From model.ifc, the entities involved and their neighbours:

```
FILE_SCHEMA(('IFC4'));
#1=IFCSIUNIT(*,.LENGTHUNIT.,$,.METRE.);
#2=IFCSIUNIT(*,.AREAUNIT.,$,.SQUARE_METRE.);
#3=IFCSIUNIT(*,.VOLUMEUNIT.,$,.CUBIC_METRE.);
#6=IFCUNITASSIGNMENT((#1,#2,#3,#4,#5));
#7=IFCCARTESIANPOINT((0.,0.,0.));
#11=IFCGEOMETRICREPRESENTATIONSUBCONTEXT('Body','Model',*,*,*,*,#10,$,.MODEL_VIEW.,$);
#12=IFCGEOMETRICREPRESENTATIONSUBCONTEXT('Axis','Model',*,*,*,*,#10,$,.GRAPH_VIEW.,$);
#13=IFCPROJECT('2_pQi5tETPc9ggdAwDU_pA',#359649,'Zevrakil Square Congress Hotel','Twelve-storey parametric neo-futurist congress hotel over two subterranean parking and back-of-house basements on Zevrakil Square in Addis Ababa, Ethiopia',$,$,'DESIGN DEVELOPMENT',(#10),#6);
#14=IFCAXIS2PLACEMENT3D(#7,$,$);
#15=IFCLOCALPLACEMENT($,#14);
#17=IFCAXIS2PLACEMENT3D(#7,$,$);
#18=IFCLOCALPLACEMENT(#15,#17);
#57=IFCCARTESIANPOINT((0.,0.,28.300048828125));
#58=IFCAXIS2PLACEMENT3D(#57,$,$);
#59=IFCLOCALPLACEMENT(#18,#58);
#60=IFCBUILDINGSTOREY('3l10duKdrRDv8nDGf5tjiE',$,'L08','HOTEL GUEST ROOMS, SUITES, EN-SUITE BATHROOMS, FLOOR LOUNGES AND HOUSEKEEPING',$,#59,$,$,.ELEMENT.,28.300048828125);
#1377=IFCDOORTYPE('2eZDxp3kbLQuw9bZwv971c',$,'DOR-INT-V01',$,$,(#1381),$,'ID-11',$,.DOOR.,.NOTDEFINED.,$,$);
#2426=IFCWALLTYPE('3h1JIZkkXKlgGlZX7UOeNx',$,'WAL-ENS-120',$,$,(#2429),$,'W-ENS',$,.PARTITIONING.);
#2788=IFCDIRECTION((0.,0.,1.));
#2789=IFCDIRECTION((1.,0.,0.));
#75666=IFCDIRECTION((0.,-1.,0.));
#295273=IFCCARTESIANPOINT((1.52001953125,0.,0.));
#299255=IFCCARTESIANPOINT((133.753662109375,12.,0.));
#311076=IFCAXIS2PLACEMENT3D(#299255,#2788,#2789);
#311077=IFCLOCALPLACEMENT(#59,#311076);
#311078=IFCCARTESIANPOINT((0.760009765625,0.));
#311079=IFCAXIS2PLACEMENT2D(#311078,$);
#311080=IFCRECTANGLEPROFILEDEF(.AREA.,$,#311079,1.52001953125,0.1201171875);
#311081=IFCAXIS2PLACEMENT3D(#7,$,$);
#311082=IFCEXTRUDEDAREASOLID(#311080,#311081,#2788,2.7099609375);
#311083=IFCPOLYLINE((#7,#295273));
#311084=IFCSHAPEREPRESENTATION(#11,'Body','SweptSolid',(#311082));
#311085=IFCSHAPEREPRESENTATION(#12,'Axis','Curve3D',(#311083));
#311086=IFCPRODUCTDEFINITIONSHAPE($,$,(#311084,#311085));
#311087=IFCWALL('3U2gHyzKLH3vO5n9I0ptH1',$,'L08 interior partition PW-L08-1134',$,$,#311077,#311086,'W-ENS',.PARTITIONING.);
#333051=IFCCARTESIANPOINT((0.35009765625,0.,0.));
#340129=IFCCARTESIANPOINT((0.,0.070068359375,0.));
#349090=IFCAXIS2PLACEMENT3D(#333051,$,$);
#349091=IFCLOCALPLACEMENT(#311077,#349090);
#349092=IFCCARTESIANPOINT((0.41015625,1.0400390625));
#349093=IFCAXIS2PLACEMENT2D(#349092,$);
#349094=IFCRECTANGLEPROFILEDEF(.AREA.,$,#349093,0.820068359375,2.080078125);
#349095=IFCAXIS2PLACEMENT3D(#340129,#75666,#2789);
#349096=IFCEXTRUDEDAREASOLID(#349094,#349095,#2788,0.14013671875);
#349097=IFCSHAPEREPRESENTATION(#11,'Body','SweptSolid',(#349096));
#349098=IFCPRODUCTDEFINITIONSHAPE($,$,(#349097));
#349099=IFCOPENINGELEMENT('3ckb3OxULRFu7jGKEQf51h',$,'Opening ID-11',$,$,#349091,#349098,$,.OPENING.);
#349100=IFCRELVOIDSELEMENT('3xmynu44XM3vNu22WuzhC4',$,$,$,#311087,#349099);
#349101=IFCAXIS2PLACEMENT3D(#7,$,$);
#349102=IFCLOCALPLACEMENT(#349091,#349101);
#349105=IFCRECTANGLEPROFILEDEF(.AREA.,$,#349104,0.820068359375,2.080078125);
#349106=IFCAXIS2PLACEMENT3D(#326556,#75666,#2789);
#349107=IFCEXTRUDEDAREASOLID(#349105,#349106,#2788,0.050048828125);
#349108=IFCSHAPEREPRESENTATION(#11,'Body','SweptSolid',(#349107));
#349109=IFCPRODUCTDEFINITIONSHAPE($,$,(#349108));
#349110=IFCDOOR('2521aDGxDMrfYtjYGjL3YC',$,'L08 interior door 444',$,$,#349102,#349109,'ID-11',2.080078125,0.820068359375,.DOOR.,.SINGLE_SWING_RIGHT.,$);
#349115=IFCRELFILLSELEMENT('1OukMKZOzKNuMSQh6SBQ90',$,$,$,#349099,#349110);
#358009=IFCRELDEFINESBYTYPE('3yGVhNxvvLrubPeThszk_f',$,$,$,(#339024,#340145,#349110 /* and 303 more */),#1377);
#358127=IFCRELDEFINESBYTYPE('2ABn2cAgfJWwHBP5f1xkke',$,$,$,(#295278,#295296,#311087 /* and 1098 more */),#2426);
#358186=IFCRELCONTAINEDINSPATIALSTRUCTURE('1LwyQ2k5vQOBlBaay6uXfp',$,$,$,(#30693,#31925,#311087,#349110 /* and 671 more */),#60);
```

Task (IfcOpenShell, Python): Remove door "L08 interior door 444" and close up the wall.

```python
import ifcopenshell
import ifcopenshell.api.feature
import ifcopenshell.api.root
import ifcopenshell.geom
import ifcopenshell.util.shape

model = ifcopenshell.open("model.ifc")
settings = ifcopenshell.geom.settings()


def volume(element):
    """Net volume in cubic metres, openings subtracted."""
    shape = ifcopenshell.geom.create_shape(settings, element)
    return ifcopenshell.util.shape.get_volume(shape.geometry)


door = model.by_guid("2521aDGxDMrfYtjYGjL3YC")
opening = door.FillsVoids[0].RelatingOpeningElement
wall = opening.VoidsElements[0].RelatingBuildingElement
before = volume(wall)

ifcopenshell.api.root.remove_product(model, product=door)
ifcopenshell.api.feature.remove_feature(model, feature=opening)

after = volume(wall)

print(f"wall volume {before:.3f} -> {after:.3f} m3")

model.write("model_edited.ifc")
```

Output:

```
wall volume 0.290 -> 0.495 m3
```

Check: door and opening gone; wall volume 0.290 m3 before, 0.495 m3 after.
